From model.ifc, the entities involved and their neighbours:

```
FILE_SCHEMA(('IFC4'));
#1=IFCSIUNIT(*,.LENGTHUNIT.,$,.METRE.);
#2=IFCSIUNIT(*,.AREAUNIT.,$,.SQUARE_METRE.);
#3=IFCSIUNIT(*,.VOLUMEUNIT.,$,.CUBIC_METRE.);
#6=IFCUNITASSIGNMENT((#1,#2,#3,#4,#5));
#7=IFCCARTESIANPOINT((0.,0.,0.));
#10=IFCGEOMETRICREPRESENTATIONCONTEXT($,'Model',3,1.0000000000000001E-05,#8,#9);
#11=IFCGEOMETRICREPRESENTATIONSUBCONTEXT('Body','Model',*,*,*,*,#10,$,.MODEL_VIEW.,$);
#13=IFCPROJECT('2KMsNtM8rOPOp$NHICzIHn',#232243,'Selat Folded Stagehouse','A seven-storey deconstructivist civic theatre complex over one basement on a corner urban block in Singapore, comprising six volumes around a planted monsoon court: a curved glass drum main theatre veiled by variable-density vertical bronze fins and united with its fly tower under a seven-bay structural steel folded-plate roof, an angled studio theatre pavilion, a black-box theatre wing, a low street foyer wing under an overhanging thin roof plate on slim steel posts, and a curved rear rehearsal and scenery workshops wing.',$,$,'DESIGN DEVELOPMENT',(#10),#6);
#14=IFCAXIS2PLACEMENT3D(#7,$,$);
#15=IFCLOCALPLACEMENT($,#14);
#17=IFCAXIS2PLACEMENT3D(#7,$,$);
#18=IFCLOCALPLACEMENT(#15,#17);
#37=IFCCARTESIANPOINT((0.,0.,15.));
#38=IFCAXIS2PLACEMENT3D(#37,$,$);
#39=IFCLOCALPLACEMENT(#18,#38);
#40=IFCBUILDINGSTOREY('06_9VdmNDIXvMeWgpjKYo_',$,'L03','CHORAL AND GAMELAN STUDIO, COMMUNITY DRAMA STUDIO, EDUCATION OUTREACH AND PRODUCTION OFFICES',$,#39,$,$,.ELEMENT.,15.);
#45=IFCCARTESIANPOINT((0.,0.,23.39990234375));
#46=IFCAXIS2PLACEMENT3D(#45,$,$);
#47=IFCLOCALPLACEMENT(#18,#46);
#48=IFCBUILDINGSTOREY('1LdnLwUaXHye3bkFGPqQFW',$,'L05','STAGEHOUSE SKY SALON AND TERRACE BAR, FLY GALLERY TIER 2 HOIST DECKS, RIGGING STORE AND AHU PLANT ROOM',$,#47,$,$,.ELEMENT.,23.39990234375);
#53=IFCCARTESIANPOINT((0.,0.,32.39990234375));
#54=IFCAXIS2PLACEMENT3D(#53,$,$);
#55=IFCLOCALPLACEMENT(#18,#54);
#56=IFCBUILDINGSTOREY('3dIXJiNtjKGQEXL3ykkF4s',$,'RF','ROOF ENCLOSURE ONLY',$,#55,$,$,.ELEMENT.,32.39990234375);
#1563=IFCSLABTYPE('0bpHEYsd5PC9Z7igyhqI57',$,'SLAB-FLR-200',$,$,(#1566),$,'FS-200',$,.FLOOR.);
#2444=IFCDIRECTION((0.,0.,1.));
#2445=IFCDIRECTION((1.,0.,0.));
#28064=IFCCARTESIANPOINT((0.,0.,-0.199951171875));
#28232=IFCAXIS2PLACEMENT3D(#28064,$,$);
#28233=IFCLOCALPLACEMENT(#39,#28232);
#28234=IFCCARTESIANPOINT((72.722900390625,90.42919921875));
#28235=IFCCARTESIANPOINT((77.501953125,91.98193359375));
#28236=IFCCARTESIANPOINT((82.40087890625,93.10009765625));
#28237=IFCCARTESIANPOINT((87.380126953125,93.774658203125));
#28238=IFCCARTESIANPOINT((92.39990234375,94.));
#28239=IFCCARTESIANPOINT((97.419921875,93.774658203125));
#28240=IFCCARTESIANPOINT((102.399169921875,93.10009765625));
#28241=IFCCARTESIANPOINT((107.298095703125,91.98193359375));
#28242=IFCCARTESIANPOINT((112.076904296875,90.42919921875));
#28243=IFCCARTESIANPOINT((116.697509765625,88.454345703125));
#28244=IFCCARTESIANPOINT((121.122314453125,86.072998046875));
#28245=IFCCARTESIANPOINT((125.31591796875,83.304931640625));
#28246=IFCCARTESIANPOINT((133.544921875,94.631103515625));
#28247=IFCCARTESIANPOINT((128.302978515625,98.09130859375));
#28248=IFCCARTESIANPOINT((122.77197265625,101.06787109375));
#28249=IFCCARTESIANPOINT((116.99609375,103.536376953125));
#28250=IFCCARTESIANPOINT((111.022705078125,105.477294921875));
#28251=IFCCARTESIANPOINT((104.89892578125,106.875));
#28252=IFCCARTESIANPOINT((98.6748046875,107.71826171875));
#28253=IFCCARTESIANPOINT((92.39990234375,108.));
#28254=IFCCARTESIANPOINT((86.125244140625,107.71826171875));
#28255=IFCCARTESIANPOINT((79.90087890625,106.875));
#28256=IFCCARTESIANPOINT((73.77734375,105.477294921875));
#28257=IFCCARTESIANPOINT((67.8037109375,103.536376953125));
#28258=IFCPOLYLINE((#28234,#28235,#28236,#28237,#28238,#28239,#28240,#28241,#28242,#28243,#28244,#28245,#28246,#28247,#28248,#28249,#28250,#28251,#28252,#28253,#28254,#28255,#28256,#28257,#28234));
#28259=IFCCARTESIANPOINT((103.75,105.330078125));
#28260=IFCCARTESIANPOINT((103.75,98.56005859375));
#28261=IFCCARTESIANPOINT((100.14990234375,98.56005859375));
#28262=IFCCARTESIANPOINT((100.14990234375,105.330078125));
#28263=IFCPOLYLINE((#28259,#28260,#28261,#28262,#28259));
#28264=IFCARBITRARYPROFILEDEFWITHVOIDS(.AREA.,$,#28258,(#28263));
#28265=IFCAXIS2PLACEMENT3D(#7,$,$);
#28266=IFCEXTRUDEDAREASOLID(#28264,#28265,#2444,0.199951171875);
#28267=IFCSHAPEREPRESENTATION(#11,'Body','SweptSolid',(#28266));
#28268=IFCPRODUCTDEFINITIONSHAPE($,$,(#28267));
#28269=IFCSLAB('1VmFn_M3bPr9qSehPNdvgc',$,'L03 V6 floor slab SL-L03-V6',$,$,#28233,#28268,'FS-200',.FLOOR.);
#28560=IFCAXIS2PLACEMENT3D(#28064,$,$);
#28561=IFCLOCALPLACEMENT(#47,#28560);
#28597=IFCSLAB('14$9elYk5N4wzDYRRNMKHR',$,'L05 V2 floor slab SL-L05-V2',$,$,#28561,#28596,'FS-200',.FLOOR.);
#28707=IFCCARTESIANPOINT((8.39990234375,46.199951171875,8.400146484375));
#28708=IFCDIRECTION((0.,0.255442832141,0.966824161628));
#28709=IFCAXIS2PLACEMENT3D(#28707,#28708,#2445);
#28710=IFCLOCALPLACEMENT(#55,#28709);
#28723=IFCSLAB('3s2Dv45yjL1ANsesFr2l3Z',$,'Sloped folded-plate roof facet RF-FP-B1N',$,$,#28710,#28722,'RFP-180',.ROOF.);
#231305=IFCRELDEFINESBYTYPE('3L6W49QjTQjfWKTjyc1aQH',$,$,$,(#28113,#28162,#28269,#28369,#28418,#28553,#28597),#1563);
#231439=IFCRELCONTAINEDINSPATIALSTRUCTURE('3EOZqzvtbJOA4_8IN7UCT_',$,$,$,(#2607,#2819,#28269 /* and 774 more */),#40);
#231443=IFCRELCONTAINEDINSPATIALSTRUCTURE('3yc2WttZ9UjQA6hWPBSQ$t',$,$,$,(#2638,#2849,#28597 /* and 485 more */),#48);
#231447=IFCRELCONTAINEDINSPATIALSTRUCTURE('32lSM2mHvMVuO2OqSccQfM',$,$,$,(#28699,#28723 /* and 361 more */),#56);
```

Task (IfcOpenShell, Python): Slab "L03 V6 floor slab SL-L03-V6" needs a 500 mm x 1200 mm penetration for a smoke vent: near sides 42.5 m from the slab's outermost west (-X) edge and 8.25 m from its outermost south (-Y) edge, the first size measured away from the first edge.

```python
import numpy as np
import ifcopenshell
import ifcopenshell.api.feature
import ifcopenshell.api.geometry
import ifcopenshell.api.root
import ifcopenshell.geom
import ifcopenshell.util.placement
import ifcopenshell.util.representation
import ifcopenshell.util.shape
import ifcopenshell.util.unit

model = ifcopenshell.open("model.ifc")
unit_scale = ifcopenshell.util.unit.calculate_unit_scale(model)
settings = ifcopenshell.geom.settings()


def volume(element):
    """Net volume in cubic metres, openings subtracted."""
    shape = ifcopenshell.geom.create_shape(settings, element)
    return ifcopenshell.util.shape.get_volume(shape.geometry)


slab = model.by_guid("1VmFn_M3bPr9qSehPNdvgc")
before = volume(slab)

# Extent in the slab's own axes, in metres. The edges named are its -X and -Y sides.
slab_shape = ifcopenshell.geom.create_shape(settings, slab)
vertices = ifcopenshell.util.shape.get_vertices(slab_shape.geometry)
x_min, y_min, bottom = vertices.min(axis=0)
top = vertices[:, 2].max()

opening = ifcopenshell.api.root.create_entity(model, ifc_class="IfcOpeningElement", name="Smoke vent opening", predefined_type="OPENING")
context = ifcopenshell.util.representation.get_context(model, "Model", "Body", "MODEL_VIEW")
width, depth = 0.5, 1.2
outline = [(0.0, 0.0), (width, 0.0), (width, depth), (0.0, depth), (0.0, 0.0)]
# Overshoot both faces by 50 mm so the cut is clean.
shape = ifcopenshell.api.geometry.add_slab_representation(
    model, context=context, depth=top - bottom + 0.1, polyline=outline
)
ifcopenshell.api.geometry.assign_representation(model, product=opening, representation=shape)

matrix = ifcopenshell.util.placement.get_local_placement(slab.ObjectPlacement)
matrix[:, 3] = matrix @ np.append(np.array([x_min + 42.5, y_min + 8.25, bottom - 0.05]) / unit_scale, 1.0)
ifcopenshell.api.geometry.edit_object_placement(model, product=opening, matrix=matrix, is_si=False)
ifcopenshell.api.feature.add_feature(model, feature=opening, element=slab)

after = volume(slab)

print(f"slab volume {before:.3f} -> {after:.3f} m3")

model.write("model_v2.ifc")
```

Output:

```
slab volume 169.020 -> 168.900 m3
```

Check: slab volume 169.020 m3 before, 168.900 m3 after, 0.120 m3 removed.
